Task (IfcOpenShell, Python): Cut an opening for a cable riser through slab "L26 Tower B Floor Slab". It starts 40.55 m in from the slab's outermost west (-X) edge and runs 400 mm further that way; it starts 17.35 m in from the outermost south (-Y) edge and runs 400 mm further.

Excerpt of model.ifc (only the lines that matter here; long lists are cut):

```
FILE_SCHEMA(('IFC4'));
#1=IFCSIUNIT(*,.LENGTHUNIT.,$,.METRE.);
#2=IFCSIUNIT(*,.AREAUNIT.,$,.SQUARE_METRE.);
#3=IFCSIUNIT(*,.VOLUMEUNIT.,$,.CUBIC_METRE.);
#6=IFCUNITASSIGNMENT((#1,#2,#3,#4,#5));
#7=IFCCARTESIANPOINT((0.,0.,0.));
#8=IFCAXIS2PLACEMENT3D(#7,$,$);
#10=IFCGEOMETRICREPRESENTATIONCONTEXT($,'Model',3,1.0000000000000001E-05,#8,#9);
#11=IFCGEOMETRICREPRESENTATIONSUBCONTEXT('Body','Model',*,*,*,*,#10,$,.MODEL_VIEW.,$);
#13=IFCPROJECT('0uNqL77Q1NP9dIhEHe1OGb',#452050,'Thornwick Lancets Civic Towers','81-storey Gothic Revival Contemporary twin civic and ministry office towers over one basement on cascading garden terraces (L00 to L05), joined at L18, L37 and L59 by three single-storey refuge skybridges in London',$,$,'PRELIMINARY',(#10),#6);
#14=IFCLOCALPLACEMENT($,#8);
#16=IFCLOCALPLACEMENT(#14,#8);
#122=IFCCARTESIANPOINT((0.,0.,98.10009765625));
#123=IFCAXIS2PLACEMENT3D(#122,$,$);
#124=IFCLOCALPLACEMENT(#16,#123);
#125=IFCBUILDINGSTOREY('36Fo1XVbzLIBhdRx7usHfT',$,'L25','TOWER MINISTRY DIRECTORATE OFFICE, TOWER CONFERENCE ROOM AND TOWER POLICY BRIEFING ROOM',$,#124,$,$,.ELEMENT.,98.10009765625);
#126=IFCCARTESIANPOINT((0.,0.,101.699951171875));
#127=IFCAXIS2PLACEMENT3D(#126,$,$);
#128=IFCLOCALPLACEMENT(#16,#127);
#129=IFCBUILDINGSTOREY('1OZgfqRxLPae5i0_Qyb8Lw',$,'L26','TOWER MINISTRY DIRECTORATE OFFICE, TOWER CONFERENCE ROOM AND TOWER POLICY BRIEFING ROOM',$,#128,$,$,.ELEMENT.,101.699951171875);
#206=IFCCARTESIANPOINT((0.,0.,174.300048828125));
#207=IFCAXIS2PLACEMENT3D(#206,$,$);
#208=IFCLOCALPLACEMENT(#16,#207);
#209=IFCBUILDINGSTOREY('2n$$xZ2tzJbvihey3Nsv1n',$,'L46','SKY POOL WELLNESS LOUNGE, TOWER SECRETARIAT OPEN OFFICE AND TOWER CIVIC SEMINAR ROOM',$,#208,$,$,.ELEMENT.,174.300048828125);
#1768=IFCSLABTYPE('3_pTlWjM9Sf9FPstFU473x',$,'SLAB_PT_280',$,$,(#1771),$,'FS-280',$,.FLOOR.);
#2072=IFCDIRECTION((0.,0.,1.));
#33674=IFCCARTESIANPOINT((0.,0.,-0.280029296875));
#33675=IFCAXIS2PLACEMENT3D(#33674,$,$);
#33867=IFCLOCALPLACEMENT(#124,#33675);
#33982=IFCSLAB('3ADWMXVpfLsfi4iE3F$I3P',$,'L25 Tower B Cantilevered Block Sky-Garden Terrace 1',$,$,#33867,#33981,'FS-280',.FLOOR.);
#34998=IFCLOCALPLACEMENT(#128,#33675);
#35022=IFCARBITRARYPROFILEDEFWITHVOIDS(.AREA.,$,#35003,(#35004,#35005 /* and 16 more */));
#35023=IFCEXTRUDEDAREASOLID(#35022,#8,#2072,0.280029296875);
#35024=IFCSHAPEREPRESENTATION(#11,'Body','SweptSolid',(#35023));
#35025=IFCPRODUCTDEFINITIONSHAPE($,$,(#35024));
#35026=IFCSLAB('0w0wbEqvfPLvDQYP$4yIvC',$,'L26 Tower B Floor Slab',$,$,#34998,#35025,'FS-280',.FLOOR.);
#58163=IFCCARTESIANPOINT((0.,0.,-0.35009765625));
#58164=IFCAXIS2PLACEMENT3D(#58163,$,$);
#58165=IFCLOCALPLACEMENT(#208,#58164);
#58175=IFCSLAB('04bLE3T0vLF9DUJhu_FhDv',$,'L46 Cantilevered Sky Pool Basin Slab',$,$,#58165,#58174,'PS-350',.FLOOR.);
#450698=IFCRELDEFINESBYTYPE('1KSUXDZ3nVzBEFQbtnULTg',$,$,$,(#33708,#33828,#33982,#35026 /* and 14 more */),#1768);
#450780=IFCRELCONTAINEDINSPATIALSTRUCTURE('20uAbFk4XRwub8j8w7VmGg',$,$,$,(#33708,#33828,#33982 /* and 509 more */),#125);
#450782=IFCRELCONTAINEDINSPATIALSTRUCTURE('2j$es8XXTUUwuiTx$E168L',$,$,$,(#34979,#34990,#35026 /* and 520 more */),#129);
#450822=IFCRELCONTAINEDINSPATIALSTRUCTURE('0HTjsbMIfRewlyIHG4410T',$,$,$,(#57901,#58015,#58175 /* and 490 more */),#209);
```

```python
import numpy as np
import ifcopenshell
import ifcopenshell.api.feature
import ifcopenshell.api.geometry
import ifcopenshell.api.root
import ifcopenshell.geom
import ifcopenshell.util.placement
import ifcopenshell.util.representation
import ifcopenshell.util.shape
import ifcopenshell.util.unit

model = ifcopenshell.open("model.ifc")
unit_scale = ifcopenshell.util.unit.calculate_unit_scale(model)
settings = ifcopenshell.geom.settings()


def volume(element):
    """Net volume in cubic metres, openings subtracted."""
    shape = ifcopenshell.geom.create_shape(settings, element)
    return ifcopenshell.util.shape.get_volume(shape.geometry)


slab = model.by_guid("0w0wbEqvfPLvDQYP$4yIvC")
before = volume(slab)

# Extent in the slab's own axes, in metres. The edges named are its -X and -Y sides.
slab_shape = ifcopenshell.geom.create_shape(settings, slab)
vertices = ifcopenshell.util.shape.get_vertices(slab_shape.geometry)
x_min, y_min, bottom = vertices.min(axis=0)
top = vertices[:, 2].max()

opening = ifcopenshell.api.root.create_entity(model, ifc_class="IfcOpeningElement", name="Cable riser opening", predefined_type="OPENING")
context = ifcopenshell.util.representation.get_context(model, "Model", "Body", "MODEL_VIEW")
width, depth = 0.4, 0.4
outline = [(0.0, 0.0), (width, 0.0), (width, depth), (0.0, depth), (0.0, 0.0)]
# Overshoot both faces by 50 mm so the cut is clean.
shape = ifcopenshell.api.geometry.add_slab_representation(
    model, context=context, depth=top - bottom + 0.1, polyline=outline
)
ifcopenshell.api.geometry.assign_representation(model, product=opening, representation=shape)

matrix = ifcopenshell.util.placement.get_local_placement(slab.ObjectPlacement)
matrix[:, 3] = matrix @ np.append(np.array([x_min + 40.55, y_min + 17.35, bottom - 0.05]) / unit_scale, 1.0)
ifcopenshell.api.geometry.edit_object_placement(model, product=opening, matrix=matrix, is_si=False)
ifcopenshell.api.feature.add_feature(model, feature=opening, element=slab)

after = volume(slab)

print(f"slab volume {before:.3f} -> {after:.3f} m3")

model.write("model_updated.ifc")
```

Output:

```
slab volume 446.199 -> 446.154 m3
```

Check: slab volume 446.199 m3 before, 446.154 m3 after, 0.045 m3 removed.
